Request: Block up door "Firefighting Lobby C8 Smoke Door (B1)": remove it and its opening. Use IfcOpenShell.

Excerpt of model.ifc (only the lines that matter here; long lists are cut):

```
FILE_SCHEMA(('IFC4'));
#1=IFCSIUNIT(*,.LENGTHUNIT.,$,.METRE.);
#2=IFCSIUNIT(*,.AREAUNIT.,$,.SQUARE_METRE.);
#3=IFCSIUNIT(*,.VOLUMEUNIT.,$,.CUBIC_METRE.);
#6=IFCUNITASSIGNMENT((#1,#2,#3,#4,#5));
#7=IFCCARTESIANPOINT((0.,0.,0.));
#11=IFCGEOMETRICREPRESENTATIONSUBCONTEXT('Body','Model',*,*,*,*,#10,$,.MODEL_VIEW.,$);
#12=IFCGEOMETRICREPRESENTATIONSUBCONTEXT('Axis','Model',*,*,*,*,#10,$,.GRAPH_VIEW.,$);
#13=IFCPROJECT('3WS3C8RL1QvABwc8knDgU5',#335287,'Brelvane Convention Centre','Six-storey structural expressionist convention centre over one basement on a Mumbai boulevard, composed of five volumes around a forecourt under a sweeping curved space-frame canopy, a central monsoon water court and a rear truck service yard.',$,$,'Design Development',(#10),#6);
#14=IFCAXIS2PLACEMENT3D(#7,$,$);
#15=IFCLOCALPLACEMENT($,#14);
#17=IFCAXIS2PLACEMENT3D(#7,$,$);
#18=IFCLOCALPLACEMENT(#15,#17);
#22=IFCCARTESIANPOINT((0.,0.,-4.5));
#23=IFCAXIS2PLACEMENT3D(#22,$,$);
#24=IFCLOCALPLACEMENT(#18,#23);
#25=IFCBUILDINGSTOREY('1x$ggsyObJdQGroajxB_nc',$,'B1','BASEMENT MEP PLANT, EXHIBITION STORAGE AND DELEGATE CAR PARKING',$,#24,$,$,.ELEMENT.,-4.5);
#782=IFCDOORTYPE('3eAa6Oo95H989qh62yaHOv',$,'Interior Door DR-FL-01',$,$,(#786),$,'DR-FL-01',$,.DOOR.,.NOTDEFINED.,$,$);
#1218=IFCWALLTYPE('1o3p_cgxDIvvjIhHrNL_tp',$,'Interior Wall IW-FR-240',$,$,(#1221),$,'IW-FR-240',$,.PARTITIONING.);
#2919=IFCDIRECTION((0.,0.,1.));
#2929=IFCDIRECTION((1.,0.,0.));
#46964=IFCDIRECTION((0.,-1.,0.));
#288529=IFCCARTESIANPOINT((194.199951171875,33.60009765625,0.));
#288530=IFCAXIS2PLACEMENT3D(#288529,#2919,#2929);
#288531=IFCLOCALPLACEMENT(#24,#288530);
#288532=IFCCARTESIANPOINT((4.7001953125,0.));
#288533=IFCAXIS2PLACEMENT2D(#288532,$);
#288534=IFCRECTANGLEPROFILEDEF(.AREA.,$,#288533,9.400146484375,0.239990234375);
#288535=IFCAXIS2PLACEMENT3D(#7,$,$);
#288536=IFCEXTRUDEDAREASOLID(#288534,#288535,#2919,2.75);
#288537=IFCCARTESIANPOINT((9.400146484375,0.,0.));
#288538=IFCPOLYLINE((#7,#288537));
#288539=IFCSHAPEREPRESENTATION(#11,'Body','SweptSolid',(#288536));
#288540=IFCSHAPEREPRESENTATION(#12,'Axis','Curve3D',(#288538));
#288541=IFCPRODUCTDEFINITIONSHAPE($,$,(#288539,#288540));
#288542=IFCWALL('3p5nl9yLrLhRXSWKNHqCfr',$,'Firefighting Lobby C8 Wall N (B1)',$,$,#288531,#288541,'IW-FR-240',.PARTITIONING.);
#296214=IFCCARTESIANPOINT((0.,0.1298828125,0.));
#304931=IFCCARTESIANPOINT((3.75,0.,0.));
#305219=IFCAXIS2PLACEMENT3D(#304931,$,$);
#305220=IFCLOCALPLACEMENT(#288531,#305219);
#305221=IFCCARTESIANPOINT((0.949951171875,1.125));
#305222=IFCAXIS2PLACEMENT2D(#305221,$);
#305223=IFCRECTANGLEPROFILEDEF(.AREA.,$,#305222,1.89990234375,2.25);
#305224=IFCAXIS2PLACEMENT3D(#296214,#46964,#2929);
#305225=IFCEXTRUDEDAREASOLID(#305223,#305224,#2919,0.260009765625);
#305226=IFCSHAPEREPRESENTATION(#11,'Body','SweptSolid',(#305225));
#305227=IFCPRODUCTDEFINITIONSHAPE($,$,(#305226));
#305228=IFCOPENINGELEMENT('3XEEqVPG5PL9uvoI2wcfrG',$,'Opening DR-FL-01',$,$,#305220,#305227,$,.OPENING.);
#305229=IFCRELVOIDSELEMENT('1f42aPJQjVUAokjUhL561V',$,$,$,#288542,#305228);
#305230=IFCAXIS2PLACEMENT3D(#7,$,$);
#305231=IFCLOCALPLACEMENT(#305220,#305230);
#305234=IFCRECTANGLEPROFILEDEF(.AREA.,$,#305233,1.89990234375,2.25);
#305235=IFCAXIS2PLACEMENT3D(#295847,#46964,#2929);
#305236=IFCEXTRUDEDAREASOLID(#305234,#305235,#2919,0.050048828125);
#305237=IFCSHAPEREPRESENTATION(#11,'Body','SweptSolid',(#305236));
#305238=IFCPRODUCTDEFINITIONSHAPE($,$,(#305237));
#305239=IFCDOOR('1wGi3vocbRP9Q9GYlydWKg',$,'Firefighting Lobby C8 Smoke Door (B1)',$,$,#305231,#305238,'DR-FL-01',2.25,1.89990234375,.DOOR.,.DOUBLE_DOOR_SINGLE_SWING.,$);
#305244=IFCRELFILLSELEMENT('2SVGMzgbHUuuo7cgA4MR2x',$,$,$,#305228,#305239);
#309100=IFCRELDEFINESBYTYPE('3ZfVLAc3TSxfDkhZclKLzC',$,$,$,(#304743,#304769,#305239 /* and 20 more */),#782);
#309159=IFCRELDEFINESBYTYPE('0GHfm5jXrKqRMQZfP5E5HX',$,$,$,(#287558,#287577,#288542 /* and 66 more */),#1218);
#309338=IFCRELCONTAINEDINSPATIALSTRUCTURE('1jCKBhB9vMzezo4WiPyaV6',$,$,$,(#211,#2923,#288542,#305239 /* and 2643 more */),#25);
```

```python
import ifcopenshell
import ifcopenshell.api.feature
import ifcopenshell.api.root
import ifcopenshell.geom
import ifcopenshell.util.shape

model = ifcopenshell.open("model.ifc")
settings = ifcopenshell.geom.settings()


def volume(element):
    """Net volume in cubic metres, openings subtracted."""
    shape = ifcopenshell.geom.create_shape(settings, element)
    return ifcopenshell.util.shape.get_volume(shape.geometry)


door = model.by_guid("1wGi3vocbRP9Q9GYlydWKg")
opening = door.FillsVoids[0].RelatingOpeningElement
wall = opening.VoidsElements[0].RelatingBuildingElement
before = volume(wall)

ifcopenshell.api.root.remove_product(model, product=door)
ifcopenshell.api.feature.remove_feature(model, feature=opening)

after = volume(wall)

print(f"wall volume {before:.3f} -> {after:.3f} m3")

model.write("model_v2.ifc")
```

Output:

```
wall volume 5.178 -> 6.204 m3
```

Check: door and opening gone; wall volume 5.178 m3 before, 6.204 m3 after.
